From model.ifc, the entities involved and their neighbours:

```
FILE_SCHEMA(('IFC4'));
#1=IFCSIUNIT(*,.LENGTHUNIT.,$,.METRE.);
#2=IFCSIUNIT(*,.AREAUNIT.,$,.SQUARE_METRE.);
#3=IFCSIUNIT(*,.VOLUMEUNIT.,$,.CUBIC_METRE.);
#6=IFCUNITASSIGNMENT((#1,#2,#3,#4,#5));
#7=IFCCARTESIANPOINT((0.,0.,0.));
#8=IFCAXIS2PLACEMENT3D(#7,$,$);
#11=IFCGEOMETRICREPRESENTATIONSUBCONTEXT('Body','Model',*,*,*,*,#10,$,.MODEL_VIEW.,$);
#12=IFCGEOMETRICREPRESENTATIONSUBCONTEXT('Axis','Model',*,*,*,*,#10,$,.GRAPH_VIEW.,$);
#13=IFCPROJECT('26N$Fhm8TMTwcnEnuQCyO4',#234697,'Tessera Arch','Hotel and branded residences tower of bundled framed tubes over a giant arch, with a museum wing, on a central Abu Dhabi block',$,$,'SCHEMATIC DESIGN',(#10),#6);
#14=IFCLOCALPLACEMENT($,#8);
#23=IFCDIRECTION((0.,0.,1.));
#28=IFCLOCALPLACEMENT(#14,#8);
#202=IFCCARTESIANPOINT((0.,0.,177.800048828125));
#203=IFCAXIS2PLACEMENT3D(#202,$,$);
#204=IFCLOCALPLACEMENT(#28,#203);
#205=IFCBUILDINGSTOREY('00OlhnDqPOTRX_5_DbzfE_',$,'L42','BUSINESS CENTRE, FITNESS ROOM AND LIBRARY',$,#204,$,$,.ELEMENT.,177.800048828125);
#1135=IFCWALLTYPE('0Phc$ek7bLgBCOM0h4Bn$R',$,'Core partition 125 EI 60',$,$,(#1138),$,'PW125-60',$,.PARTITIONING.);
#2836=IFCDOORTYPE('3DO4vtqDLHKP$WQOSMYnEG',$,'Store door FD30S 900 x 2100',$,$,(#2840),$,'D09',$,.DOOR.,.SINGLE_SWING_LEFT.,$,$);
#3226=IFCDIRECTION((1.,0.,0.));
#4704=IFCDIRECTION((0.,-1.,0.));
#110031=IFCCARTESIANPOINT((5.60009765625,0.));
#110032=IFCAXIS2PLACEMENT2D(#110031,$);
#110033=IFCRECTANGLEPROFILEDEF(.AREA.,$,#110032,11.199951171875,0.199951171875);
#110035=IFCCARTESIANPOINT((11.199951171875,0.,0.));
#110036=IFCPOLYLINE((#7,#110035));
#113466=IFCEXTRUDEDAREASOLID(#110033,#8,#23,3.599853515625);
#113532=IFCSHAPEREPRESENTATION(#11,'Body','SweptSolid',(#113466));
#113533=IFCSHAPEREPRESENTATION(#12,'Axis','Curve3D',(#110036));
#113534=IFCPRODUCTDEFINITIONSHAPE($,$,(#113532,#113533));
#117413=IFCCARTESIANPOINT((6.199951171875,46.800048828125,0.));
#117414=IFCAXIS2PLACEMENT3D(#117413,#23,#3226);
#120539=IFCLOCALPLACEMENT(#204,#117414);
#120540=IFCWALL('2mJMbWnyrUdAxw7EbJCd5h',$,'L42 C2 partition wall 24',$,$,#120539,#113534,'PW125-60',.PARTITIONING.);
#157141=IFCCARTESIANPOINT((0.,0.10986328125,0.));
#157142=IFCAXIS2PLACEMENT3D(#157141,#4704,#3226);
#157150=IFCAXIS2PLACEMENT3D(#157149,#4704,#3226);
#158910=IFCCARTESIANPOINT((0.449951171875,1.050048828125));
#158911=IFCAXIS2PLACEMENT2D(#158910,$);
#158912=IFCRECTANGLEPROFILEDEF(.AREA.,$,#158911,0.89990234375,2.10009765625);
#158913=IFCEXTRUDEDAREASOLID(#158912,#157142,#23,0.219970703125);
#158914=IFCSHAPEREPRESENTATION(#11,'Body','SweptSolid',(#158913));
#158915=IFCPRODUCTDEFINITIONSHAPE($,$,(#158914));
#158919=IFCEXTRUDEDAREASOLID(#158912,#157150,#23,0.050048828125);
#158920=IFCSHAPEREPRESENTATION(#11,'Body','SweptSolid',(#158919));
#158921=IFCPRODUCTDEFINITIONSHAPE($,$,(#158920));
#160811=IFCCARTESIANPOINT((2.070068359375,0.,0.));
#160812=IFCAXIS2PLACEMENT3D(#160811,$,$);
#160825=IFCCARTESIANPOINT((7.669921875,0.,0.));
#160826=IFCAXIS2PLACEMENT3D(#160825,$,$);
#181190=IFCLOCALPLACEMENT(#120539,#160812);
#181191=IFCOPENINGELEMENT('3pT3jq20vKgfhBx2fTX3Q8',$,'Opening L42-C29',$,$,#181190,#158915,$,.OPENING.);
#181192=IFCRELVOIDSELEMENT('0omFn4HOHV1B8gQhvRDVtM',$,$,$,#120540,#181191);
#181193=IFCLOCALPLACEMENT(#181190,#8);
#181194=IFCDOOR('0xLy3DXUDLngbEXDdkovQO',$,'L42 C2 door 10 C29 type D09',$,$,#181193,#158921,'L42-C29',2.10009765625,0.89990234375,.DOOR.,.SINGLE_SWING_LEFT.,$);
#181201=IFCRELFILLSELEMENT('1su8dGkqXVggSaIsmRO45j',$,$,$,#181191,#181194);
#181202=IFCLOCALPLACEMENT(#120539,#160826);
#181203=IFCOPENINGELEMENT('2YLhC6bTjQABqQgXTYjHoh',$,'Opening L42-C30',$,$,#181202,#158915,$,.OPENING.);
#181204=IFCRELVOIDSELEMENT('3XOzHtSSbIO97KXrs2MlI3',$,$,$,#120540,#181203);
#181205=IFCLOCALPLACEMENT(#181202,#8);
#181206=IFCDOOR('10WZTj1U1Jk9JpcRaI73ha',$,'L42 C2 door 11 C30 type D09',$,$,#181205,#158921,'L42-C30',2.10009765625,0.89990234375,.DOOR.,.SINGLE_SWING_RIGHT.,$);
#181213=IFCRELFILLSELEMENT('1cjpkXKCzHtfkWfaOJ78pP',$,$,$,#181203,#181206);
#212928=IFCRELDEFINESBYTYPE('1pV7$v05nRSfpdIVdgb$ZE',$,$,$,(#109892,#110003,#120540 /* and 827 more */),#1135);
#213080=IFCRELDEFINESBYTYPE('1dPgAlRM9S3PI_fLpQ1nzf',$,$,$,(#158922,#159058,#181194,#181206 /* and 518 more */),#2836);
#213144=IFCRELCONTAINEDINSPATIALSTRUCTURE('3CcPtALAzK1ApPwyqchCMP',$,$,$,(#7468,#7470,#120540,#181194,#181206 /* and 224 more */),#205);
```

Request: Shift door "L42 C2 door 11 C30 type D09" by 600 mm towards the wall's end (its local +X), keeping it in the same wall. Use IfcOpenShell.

```python
import ifcopenshell
import ifcopenshell.api.geometry
import ifcopenshell.util.placement

model = ifcopenshell.open("model.ifc")

door = model.by_guid("10WZTj1U1Jk9JpcRaI73ha")
opening = door.FillsVoids[0].RelatingOpeningElement
wall = opening.VoidsElements[0].RelatingBuildingElement

wall_matrix = ifcopenshell.util.placement.get_local_placement(wall.ObjectPlacement)
shift = wall_matrix[:3, 0] * 0.6
before = ifcopenshell.util.placement.get_local_placement(door.ObjectPlacement)[:3, 3].copy()

# The door is placed relative to its opening, so it follows when the opening moves.
matrix = ifcopenshell.util.placement.get_local_placement(opening.ObjectPlacement)
matrix[:3, 3] += shift
ifcopenshell.api.geometry.edit_object_placement(
    model, product=opening, matrix=matrix, is_si=False, should_transform_children=True
)

after = ifcopenshell.util.placement.get_local_placement(door.ObjectPlacement)[:3, 3]
print("door moved by", (after - before).round(3) + 0.0)

model.write("model_edited.ifc")
```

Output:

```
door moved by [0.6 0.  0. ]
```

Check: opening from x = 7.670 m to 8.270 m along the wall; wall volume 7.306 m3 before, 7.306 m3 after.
